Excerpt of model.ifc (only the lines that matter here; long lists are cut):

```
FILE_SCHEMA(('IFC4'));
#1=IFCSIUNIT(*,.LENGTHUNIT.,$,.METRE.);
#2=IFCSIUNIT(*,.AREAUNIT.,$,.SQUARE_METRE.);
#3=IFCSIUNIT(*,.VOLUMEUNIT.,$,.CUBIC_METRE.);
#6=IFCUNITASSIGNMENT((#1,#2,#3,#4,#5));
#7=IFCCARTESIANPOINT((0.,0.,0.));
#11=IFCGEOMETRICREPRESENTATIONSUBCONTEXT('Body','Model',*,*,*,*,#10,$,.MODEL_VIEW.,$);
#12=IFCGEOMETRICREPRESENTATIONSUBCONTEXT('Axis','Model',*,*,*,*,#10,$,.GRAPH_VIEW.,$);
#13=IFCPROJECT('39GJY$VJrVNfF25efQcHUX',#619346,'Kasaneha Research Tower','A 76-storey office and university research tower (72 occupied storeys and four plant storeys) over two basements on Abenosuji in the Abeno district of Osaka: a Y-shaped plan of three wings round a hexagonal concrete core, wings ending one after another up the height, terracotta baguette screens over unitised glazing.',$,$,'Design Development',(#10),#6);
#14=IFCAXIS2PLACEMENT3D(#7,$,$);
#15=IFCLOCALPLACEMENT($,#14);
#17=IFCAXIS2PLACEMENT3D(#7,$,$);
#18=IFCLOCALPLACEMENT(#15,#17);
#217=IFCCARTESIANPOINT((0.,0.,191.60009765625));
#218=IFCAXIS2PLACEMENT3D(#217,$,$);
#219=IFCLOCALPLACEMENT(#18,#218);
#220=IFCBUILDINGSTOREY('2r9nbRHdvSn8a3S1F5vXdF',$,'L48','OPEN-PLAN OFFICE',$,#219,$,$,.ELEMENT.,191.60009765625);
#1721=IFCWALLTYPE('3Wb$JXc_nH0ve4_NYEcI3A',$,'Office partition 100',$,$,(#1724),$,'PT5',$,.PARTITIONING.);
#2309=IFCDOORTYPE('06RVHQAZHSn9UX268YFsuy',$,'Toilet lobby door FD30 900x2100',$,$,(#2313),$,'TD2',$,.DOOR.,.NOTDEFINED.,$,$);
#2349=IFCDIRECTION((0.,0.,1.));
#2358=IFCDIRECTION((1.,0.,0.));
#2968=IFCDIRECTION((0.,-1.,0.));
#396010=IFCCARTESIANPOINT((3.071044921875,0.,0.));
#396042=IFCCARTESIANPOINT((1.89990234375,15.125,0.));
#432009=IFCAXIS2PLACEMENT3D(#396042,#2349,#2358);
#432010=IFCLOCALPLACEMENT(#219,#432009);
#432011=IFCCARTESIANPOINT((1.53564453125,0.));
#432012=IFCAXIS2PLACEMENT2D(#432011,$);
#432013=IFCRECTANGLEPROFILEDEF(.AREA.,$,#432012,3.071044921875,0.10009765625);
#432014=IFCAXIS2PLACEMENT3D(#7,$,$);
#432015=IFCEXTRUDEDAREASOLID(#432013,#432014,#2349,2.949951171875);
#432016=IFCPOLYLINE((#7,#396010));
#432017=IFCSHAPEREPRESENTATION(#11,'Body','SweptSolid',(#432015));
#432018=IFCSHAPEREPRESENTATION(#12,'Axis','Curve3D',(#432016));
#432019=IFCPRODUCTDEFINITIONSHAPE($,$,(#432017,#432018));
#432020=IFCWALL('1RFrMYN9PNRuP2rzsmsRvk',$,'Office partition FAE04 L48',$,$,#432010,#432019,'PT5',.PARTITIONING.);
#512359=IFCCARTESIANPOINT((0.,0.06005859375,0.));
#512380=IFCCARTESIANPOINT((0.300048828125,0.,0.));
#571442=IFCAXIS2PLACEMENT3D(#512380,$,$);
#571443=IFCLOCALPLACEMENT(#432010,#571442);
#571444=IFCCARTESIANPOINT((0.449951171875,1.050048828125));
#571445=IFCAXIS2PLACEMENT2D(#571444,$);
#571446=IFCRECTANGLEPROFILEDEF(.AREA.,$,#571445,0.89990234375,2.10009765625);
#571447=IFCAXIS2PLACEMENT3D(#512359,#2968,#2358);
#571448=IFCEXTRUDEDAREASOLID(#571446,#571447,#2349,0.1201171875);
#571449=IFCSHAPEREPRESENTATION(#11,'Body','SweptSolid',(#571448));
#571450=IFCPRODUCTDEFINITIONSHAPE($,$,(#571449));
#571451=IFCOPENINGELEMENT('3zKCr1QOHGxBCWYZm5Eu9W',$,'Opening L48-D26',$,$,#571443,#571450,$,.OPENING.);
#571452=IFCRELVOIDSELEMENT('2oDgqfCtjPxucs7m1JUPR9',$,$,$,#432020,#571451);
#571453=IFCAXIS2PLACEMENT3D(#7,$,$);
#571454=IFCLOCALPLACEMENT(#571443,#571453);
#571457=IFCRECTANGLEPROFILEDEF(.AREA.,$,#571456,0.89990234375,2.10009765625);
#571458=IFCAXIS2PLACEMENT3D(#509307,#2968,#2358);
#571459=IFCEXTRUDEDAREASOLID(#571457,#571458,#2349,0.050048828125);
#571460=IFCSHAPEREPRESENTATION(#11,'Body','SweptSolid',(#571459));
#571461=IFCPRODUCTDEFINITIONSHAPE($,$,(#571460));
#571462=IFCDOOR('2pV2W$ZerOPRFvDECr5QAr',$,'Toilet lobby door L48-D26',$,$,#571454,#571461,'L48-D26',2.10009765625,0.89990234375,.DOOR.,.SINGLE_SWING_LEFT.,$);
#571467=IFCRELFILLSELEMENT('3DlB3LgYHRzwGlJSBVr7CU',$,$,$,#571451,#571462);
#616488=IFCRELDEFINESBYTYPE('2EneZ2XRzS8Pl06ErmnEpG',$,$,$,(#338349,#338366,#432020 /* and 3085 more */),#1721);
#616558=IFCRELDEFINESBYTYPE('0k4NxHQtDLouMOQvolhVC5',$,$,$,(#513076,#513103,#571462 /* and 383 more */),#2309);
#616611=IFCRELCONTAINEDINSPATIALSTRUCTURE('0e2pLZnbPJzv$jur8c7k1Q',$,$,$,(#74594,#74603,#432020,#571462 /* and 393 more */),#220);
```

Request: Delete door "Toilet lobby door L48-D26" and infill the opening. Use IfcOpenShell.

```python
import ifcopenshell
import ifcopenshell.api.feature
import ifcopenshell.api.root
import ifcopenshell.geom
import ifcopenshell.util.shape

model = ifcopenshell.open("model.ifc")
settings = ifcopenshell.geom.settings()


def volume(element):
    """Net volume in cubic metres, openings subtracted."""
    shape = ifcopenshell.geom.create_shape(settings, element)
    return ifcopenshell.util.shape.get_volume(shape.geometry)


door = model.by_guid("2pV2W$ZerOPRFvDECr5QAr")
opening = door.FillsVoids[0].RelatingOpeningElement
wall = opening.VoidsElements[0].RelatingBuildingElement
before = volume(wall)

ifcopenshell.api.root.remove_product(model, product=door)
ifcopenshell.api.feature.remove_feature(model, feature=opening)

after = volume(wall)

print(f"wall volume {before:.3f} -> {after:.3f} m3")

model.write("model-out.ifc")
```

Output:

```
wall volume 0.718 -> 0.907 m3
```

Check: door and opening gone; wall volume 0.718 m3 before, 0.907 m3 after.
